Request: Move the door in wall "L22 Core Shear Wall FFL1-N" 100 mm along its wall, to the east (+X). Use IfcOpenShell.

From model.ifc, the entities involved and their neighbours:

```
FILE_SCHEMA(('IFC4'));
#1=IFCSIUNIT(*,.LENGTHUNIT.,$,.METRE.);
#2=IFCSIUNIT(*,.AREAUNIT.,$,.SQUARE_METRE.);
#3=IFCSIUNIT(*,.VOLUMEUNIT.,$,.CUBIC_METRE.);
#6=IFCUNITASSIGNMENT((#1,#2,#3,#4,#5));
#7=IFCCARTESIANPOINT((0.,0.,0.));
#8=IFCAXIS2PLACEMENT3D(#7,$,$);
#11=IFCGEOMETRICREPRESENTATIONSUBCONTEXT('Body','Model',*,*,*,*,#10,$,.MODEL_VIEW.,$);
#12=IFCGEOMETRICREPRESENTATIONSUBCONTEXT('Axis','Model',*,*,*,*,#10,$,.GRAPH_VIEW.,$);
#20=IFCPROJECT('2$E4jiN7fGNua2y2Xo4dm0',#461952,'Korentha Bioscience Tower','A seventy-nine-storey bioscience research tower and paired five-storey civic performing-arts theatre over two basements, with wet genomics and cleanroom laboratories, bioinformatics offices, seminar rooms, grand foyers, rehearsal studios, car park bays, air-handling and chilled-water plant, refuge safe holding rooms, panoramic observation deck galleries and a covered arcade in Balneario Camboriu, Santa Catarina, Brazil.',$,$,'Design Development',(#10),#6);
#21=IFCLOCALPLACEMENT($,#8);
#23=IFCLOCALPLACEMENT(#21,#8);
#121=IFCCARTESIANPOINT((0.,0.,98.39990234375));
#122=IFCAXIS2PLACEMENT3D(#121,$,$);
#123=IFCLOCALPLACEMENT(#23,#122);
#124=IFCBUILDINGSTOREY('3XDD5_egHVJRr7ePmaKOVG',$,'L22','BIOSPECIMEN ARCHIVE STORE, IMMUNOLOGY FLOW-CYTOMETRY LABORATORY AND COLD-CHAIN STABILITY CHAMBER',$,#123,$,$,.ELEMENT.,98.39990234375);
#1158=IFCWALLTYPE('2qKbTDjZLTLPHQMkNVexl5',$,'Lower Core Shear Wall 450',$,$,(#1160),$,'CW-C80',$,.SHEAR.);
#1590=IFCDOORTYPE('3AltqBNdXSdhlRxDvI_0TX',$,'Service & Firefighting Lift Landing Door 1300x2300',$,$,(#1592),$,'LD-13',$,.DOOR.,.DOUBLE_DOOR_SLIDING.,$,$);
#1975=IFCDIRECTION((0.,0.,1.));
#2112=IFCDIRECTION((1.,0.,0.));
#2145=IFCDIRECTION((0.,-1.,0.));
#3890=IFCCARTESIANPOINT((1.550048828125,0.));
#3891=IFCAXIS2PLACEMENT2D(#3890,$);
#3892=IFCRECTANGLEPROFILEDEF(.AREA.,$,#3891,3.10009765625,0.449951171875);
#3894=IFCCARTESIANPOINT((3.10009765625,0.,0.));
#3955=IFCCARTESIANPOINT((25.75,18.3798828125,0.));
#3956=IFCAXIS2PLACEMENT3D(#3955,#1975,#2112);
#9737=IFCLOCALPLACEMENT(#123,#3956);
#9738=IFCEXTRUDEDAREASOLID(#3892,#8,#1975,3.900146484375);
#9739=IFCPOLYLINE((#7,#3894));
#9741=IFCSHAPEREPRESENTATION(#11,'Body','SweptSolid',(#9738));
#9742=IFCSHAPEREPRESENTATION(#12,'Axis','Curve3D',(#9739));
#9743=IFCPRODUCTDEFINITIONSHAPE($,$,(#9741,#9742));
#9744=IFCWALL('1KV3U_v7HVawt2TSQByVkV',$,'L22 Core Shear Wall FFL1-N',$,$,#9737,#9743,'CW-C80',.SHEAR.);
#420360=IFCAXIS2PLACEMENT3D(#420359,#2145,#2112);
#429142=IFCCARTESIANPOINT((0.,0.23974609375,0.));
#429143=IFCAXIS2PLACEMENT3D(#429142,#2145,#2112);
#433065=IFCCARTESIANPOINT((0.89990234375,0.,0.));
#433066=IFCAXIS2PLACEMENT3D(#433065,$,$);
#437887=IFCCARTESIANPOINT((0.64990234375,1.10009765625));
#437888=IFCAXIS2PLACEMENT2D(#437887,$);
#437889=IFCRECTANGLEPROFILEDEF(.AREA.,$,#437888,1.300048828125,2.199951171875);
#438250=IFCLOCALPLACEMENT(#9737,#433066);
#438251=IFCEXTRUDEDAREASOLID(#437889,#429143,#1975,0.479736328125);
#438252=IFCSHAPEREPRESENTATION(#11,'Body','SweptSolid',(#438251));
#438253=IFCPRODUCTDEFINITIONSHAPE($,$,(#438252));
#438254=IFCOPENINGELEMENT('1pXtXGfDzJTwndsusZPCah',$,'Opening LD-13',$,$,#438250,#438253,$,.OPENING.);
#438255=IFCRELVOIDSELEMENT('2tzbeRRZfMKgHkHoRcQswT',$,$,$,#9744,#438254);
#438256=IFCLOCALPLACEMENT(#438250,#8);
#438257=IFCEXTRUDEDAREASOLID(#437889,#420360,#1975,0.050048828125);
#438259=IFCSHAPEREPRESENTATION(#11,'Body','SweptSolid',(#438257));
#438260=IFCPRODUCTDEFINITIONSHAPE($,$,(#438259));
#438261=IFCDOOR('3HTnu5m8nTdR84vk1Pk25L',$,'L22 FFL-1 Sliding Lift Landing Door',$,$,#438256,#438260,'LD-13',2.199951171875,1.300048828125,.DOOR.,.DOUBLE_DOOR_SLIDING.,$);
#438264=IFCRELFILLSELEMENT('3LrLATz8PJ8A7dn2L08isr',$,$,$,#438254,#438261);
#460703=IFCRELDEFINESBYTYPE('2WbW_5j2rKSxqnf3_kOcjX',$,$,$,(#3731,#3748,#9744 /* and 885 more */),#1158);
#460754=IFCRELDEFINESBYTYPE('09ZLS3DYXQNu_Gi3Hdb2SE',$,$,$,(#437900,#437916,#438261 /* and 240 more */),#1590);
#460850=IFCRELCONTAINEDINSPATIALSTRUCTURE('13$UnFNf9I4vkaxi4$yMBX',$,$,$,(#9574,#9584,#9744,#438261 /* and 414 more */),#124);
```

```python
import ifcopenshell
import ifcopenshell.api.geometry
import ifcopenshell.util.placement
import ifcopenshell.util.unit

model = ifcopenshell.open("model.ifc")
unit_scale = ifcopenshell.util.unit.calculate_unit_scale(model)

door = model.by_guid("3HTnu5m8nTdR84vk1Pk25L")
opening = door.FillsVoids[0].RelatingOpeningElement
wall = opening.VoidsElements[0].RelatingBuildingElement

wall_matrix = ifcopenshell.util.placement.get_local_placement(wall.ObjectPlacement)
shift = wall_matrix[:3, 0] * 0.1 / unit_scale
before = ifcopenshell.util.placement.get_local_placement(door.ObjectPlacement)[:3, 3].copy()

# The door is placed relative to its opening, so it follows when the opening moves.
matrix = ifcopenshell.util.placement.get_local_placement(opening.ObjectPlacement)
matrix[:3, 3] += shift
ifcopenshell.api.geometry.edit_object_placement(
    model, product=opening, matrix=matrix, is_si=False, should_transform_children=True
)

after = ifcopenshell.util.placement.get_local_placement(door.ObjectPlacement)[:3, 3]
print("door moved by", (after - before).round(3) + 0.0)

model.write("model_v2.ifc")
```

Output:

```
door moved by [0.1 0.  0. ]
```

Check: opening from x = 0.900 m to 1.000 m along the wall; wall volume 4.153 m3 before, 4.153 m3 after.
